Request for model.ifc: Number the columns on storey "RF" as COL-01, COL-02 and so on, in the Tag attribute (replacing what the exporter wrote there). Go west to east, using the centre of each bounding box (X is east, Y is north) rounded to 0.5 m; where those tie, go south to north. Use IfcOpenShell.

First a look at what the model holds.

```python
import ifcopenshell
import ifcopenshell.util.element
import ifcopenshell.util.placement

model = ifcopenshell.open("model.ifc")
print(model.schema)
storey = next(s for s in model.by_type("IfcBuildingStorey") if s.Name == "RF")
columns = [e for e in ifcopenshell.util.element.get_decomposition(storey) if e.is_a("IfcColumn")]
for e in sorted(columns, key=lambda e: e.id()):
    origin = ifcopenshell.util.placement.get_local_placement(e.ObjectPlacement)[:3, 3]
    print(e.id(), e.Tag, e.Name, origin.round(2) + 0.0, sep=" | ")
```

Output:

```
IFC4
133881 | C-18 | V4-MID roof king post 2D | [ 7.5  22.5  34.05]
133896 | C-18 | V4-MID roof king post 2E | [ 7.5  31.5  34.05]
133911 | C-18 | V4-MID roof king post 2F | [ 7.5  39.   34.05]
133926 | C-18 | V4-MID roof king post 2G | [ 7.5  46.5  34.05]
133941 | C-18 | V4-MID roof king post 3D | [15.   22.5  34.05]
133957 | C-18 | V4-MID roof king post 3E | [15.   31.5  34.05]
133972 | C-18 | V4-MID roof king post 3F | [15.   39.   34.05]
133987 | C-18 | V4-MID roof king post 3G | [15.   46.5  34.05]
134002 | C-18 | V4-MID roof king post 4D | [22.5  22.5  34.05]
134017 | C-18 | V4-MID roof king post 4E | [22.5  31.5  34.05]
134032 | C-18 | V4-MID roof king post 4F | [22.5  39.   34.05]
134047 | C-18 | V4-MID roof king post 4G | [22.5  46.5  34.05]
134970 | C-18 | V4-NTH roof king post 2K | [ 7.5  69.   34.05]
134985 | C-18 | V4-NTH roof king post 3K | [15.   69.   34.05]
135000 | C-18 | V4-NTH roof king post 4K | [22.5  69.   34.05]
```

```python
import ifcopenshell
import ifcopenshell.geom
import ifcopenshell.util.element
import ifcopenshell.util.shape

model = ifcopenshell.open("model.ifc")
settings = ifcopenshell.geom.settings()
settings.set("use-world-coords", True)


def centre(element):
    shape = ifcopenshell.geom.create_shape(settings, element)
    return ifcopenshell.util.shape.get_bbox_centroid(shape.geometry)


storey = next(s for s in model.by_type("IfcBuildingStorey") if s.Name == "RF")
columns = [e for e in ifcopenshell.util.element.get_decomposition(storey) if e.is_a("IfcColumn")]

# Insertion points can sit at a corner or the storey origin, so sort by the geometry (in metres).
centres = {e: centre(e) for e in columns}
columns.sort(key=lambda e: (round(centres[e][0] / 0.5), centres[e][1]))

for i, e in enumerate(columns, start=1):
    number = f"COL-{i:02d}"
    e.Tag = number
    print(e.id(), number)

model.write("model_edited.ifc")
```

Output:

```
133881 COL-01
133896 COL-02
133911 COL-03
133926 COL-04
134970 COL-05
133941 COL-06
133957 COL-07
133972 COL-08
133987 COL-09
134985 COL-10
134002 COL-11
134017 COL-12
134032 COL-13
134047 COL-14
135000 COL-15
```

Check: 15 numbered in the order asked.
